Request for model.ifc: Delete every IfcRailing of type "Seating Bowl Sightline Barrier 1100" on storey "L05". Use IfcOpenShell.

First a look at what the model holds.

```python
import ifcopenshell
import ifcopenshell.util.element

model = ifcopenshell.open("model.ifc")
print(model.schema)
storey = next(s for s in model.by_type("IfcBuildingStorey") if s.Name == "L05")
railings = [e for e in ifcopenshell.util.element.get_decomposition(storey) if e.is_a("IfcRailing")]
seen = {}
for e in railings:
    element_type = ifcopenshell.util.element.get_type(e)
    name = element_type.Name if element_type not in (None, e) else None
    seen[name] = seen.get(name, 0) + 1
for name, count in sorted(seen.items(), key=str):
    print(count, "x", name)
```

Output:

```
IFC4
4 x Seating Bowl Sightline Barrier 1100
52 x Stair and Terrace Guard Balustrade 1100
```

```python
import ifcopenshell
import ifcopenshell.api.root
import ifcopenshell.util.element

model = ifcopenshell.open("model.ifc")

storey = next(s for s in model.by_type("IfcBuildingStorey") if s.Name == "L05")
railings = [e for e in ifcopenshell.util.element.get_decomposition(storey) if e.is_a("IfcRailing")]
targets = [e for e in railings if (t := ifcopenshell.util.element.get_type(e)) not in (None, e) and t.Name == "Seating Bowl Sightline Barrier 1100"]

for e in targets:
    ifcopenshell.api.root.remove_product(model, product=e)
print(len(targets), "removed")

model.write("model_v2.ifc")
```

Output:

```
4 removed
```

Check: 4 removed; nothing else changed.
